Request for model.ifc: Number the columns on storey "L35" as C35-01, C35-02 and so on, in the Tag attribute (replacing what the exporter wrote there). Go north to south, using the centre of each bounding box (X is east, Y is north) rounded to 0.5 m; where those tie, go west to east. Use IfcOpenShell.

First a look at what the model holds.

```python
import ifcopenshell
import ifcopenshell.util.element
import ifcopenshell.util.placement

model = ifcopenshell.open("model.ifc")
print(model.schema)
storey = next(s for s in model.by_type("IfcBuildingStorey") if s.Name == "L35")
columns = [e for e in ifcopenshell.util.element.get_decomposition(storey) if e.is_a("IfcColumn")]
for e in sorted(columns, key=lambda e: e.id()):
    origin = ifcopenshell.util.placement.get_local_placement(e.ObjectPlacement)[:3, 3]
    print(e.id(), e.Tag, e.Name, origin.round(2) + 0.0, sep=" | ")
```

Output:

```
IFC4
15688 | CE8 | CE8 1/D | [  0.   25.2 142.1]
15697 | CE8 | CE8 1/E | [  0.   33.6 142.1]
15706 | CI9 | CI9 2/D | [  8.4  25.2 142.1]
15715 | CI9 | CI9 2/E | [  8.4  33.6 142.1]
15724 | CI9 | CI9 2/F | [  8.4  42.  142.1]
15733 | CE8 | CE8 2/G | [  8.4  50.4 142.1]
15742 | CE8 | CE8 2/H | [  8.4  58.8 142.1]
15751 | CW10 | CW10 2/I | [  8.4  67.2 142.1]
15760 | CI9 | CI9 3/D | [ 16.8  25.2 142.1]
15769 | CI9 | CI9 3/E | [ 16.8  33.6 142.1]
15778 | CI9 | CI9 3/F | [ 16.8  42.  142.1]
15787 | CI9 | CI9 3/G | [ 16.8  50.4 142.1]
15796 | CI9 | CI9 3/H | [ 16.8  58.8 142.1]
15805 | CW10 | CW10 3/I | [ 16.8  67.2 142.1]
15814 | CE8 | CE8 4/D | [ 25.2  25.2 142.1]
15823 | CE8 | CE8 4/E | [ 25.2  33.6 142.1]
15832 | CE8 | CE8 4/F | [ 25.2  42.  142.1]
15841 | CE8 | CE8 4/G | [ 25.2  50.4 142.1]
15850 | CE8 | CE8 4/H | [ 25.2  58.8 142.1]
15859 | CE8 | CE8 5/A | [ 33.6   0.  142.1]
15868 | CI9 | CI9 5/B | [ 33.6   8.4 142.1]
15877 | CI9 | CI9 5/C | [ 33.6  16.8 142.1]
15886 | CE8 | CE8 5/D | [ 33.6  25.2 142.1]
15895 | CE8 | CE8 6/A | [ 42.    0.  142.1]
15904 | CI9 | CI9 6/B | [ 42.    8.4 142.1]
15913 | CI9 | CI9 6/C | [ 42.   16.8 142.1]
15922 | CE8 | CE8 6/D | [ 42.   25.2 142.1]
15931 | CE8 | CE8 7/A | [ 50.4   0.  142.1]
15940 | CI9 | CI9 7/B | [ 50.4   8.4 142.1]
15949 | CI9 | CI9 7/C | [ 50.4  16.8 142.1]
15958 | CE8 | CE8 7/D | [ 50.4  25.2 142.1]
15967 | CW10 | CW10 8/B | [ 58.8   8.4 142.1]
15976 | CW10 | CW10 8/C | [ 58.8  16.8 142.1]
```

```python
import ifcopenshell
import ifcopenshell.geom
import ifcopenshell.util.element
import ifcopenshell.util.shape

model = ifcopenshell.open("model.ifc")
settings = ifcopenshell.geom.settings()
settings.set("use-world-coords", True)


def centre(element):
    shape = ifcopenshell.geom.create_shape(settings, element)
    return ifcopenshell.util.shape.get_bbox_centroid(shape.geometry)


storey = next(s for s in model.by_type("IfcBuildingStorey") if s.Name == "L35")
columns = [e for e in ifcopenshell.util.element.get_decomposition(storey) if e.is_a("IfcColumn")]

# Insertion points can sit at a corner or the storey origin, so sort by the geometry (in metres).
centres = {e: centre(e) for e in columns}
columns.sort(key=lambda e: (-round(centres[e][1] / 0.5), centres[e][0]))

for i, e in enumerate(columns, start=1):
    number = f"C35-{i:02d}"
    e.Tag = number
    print(e.id(), number)

model.write("model-out.ifc")
```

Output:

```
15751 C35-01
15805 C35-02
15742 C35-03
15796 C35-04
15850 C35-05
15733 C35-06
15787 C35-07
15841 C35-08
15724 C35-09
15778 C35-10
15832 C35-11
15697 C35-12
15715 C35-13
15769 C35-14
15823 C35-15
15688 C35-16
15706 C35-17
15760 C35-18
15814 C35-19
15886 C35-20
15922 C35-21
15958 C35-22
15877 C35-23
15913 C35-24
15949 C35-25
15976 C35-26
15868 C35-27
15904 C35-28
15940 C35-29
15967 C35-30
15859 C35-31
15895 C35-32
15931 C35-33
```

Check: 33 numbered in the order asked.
